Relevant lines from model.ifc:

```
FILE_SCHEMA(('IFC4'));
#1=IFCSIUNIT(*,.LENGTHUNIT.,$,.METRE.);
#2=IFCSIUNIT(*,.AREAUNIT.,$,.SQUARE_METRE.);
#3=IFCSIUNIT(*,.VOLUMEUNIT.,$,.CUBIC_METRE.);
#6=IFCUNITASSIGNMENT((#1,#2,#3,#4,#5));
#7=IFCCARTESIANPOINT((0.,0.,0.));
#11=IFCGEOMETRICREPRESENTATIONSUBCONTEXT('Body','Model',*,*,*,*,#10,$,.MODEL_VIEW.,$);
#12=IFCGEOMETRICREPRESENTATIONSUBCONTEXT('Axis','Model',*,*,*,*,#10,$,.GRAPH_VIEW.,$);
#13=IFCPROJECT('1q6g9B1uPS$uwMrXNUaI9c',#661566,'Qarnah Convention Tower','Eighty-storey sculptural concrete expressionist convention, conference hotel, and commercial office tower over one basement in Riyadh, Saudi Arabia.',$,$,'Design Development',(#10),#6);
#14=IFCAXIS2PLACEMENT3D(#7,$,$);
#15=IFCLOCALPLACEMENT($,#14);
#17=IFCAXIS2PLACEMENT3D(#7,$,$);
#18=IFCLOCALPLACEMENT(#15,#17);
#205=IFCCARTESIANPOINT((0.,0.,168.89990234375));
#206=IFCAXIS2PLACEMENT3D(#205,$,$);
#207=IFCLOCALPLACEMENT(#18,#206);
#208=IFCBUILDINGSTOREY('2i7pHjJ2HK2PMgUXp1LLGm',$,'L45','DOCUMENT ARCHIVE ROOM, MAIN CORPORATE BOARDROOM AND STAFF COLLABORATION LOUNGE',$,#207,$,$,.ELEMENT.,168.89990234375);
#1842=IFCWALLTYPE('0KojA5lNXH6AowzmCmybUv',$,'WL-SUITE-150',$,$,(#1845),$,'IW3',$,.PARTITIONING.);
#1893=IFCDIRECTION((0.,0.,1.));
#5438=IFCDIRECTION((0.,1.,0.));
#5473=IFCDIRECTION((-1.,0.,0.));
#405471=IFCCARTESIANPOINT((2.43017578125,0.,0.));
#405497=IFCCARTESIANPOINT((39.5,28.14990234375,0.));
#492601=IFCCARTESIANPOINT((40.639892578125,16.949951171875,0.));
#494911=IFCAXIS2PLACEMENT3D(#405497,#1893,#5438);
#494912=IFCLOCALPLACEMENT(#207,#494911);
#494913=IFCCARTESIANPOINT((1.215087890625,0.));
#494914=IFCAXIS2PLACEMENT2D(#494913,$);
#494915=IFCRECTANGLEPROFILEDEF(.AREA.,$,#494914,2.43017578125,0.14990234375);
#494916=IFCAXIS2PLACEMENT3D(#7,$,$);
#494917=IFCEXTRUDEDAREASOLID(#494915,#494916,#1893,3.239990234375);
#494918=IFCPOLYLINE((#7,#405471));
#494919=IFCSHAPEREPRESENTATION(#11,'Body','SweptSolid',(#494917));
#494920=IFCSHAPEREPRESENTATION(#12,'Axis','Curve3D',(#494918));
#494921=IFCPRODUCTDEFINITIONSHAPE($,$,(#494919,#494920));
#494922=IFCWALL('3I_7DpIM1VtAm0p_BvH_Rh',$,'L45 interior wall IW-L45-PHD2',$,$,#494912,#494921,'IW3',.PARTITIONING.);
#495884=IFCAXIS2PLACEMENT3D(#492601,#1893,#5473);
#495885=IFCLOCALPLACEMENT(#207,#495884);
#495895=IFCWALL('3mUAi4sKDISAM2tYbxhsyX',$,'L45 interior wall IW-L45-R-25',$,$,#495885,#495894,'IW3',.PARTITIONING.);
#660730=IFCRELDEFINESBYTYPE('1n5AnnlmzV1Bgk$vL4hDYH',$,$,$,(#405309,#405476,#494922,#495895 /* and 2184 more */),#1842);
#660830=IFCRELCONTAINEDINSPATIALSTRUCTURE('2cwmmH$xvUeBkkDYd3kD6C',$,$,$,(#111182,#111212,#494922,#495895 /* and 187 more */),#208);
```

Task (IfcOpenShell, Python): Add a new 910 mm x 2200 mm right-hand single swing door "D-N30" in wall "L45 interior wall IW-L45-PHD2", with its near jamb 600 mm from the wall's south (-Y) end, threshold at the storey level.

```python
import numpy as np
import ifcopenshell
import ifcopenshell.api.feature
import ifcopenshell.api.geometry
import ifcopenshell.api.root
import ifcopenshell.api.spatial
import ifcopenshell.geom
import ifcopenshell.util.element
import ifcopenshell.util.placement
import ifcopenshell.util.representation
import ifcopenshell.util.shape
import ifcopenshell.util.unit

model = ifcopenshell.open("model.ifc")
unit_scale = ifcopenshell.util.unit.calculate_unit_scale(model)
settings = ifcopenshell.geom.settings()


def volume(element):
    """Net volume in cubic metres, openings subtracted."""
    shape = ifcopenshell.geom.create_shape(settings, element)
    return ifcopenshell.util.shape.get_volume(shape.geometry)


wall = model.by_guid("3I_7DpIM1VtAm0p_BvH_Rh")
storey = ifcopenshell.util.element.get_container(wall, ifc_class="IfcBuildingStorey")
context = ifcopenshell.util.representation.get_context(model, "Model", "Body", "MODEL_VIEW")
before = volume(wall)

width, height, from_end, sill = 0.91, 2.2, 0.6, 0.0  # metres

# The wall runs along its own X axis, and the end named is its -X end.
wall_shape = ifcopenshell.geom.create_shape(settings, wall)
x, y, z = ifcopenshell.util.shape.get_vertices(wall_shape.geometry).T
start = x.min() + from_end
face, thickness = float(y.min()), float(y.max() - y.min())
wall_matrix = ifcopenshell.util.placement.get_local_placement(wall.ObjectPlacement)
level = ifcopenshell.util.placement.get_local_placement(storey.ObjectPlacement)[2, 3]


def in_wall(x, y):
    """Placement at x, y metres in the wall's axes, at sill height."""
    matrix = wall_matrix.copy()
    matrix[:, 3] = wall_matrix @ np.array([x / unit_scale, y / unit_scale, 0.0, 1.0])
    matrix[2, 3] = level + sill / unit_scale
    return matrix


# Opening: a box that overshoots both wall faces by 50 mm.
opening = ifcopenshell.api.root.create_entity(model, ifc_class="IfcOpeningElement", predefined_type="OPENING")
box = ifcopenshell.api.geometry.add_wall_representation(
    model, context=context, length=width, height=height, thickness=thickness + 0.1
)
ifcopenshell.api.geometry.assign_representation(model, product=opening, representation=box)
ifcopenshell.api.geometry.edit_object_placement(model, product=opening, matrix=in_wall(start, face - 0.05), is_si=False)
ifcopenshell.api.feature.add_feature(model, feature=opening, element=wall)

door = ifcopenshell.api.root.create_entity(model, ifc_class="IfcDoor", name="D-N30", predefined_type="DOOR")
door.OverallWidth, door.OverallHeight = width / unit_scale, height / unit_scale
door.OperationType = "SINGLE_SWING_RIGHT"
body = ifcopenshell.api.geometry.add_door_representation(
    model,
    context=context,
    overall_width=door.OverallWidth,
    overall_height=door.OverallHeight,
    operation_type="SINGLE_SWING_RIGHT",
    lining_properties={"LiningDepth": thickness / unit_scale, "ThresholdDepth": thickness / unit_scale},
)
ifcopenshell.api.geometry.assign_representation(model, product=door, representation=body)
ifcopenshell.api.spatial.assign_container(model, products=[door], relating_structure=storey)
ifcopenshell.api.feature.add_filling(model, opening=opening, element=door)

# The lining spans the wall, so the door starts at the wall face.
ifcopenshell.api.geometry.edit_object_placement(model, product=door, matrix=in_wall(start, face), is_si=False)

after = volume(wall)

print(f"wall volume {before:.3f} -> {after:.3f} m3")

model.write("model_rev.ifc")
```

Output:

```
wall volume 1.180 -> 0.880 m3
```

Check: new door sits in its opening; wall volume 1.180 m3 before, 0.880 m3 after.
